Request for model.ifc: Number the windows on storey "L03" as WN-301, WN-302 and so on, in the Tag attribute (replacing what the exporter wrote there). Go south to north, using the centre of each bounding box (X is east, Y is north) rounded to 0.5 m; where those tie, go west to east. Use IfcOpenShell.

First a look at what the model holds.

```python
import ifcopenshell
import ifcopenshell.util.element
import ifcopenshell.util.placement

model = ifcopenshell.open("model.ifc")
print(model.schema)
storey = next(s for s in model.by_type("IfcBuildingStorey") if s.Name == "L03")
windows = [e for e in ifcopenshell.util.element.get_decomposition(storey) if e.is_a("IfcWindow")]
for e in sorted(windows, key=lambda e: e.id()):
    origin = ifcopenshell.util.placement.get_local_placement(e.ObjectPlacement)[:3, 3]
    print(e.id(), e.Tag, e.Name, origin.round(2) + 0.0, sep=" | ")
```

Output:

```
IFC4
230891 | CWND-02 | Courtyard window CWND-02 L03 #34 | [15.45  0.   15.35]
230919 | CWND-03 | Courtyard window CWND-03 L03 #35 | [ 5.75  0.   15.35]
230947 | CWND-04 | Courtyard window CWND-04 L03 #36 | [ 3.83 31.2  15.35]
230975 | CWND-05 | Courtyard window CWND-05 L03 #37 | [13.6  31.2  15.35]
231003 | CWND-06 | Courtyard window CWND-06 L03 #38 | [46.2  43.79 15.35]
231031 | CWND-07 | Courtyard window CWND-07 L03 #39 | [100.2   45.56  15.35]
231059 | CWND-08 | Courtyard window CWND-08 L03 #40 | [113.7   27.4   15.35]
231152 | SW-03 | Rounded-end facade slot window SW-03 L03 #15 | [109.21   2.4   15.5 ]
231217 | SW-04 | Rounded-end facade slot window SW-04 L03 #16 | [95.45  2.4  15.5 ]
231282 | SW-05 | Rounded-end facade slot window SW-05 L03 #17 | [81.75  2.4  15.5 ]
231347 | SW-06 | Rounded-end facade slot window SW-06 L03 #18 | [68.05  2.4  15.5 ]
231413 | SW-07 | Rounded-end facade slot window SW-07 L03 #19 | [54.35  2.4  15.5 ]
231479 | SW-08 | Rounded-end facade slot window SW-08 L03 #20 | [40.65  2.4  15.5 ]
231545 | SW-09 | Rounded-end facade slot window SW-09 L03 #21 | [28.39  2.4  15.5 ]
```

```python
import ifcopenshell
import ifcopenshell.geom
import ifcopenshell.util.element
import ifcopenshell.util.shape

model = ifcopenshell.open("model.ifc")
settings = ifcopenshell.geom.settings()
settings.set("use-world-coords", True)


def centre(element):
    shape = ifcopenshell.geom.create_shape(settings, element)
    return ifcopenshell.util.shape.get_bbox_centroid(shape.geometry)


storey = next(s for s in model.by_type("IfcBuildingStorey") if s.Name == "L03")
windows = [e for e in ifcopenshell.util.element.get_decomposition(storey) if e.is_a("IfcWindow")]

# Insertion points can sit at a corner or the storey origin, so sort by the geometry (in metres).
centres = {e: centre(e) for e in windows}
windows.sort(key=lambda e: (round(centres[e][1] / 0.5), centres[e][0]))

for i, e in enumerate(windows, start=1):
    number = f"WN-3{i:02d}"
    e.Tag = number
    print(e.id(), number)

model.write("model_edited.ifc")
```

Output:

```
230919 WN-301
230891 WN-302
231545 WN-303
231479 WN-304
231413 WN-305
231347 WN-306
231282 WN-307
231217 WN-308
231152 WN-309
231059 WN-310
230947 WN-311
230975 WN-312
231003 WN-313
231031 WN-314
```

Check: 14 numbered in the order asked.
